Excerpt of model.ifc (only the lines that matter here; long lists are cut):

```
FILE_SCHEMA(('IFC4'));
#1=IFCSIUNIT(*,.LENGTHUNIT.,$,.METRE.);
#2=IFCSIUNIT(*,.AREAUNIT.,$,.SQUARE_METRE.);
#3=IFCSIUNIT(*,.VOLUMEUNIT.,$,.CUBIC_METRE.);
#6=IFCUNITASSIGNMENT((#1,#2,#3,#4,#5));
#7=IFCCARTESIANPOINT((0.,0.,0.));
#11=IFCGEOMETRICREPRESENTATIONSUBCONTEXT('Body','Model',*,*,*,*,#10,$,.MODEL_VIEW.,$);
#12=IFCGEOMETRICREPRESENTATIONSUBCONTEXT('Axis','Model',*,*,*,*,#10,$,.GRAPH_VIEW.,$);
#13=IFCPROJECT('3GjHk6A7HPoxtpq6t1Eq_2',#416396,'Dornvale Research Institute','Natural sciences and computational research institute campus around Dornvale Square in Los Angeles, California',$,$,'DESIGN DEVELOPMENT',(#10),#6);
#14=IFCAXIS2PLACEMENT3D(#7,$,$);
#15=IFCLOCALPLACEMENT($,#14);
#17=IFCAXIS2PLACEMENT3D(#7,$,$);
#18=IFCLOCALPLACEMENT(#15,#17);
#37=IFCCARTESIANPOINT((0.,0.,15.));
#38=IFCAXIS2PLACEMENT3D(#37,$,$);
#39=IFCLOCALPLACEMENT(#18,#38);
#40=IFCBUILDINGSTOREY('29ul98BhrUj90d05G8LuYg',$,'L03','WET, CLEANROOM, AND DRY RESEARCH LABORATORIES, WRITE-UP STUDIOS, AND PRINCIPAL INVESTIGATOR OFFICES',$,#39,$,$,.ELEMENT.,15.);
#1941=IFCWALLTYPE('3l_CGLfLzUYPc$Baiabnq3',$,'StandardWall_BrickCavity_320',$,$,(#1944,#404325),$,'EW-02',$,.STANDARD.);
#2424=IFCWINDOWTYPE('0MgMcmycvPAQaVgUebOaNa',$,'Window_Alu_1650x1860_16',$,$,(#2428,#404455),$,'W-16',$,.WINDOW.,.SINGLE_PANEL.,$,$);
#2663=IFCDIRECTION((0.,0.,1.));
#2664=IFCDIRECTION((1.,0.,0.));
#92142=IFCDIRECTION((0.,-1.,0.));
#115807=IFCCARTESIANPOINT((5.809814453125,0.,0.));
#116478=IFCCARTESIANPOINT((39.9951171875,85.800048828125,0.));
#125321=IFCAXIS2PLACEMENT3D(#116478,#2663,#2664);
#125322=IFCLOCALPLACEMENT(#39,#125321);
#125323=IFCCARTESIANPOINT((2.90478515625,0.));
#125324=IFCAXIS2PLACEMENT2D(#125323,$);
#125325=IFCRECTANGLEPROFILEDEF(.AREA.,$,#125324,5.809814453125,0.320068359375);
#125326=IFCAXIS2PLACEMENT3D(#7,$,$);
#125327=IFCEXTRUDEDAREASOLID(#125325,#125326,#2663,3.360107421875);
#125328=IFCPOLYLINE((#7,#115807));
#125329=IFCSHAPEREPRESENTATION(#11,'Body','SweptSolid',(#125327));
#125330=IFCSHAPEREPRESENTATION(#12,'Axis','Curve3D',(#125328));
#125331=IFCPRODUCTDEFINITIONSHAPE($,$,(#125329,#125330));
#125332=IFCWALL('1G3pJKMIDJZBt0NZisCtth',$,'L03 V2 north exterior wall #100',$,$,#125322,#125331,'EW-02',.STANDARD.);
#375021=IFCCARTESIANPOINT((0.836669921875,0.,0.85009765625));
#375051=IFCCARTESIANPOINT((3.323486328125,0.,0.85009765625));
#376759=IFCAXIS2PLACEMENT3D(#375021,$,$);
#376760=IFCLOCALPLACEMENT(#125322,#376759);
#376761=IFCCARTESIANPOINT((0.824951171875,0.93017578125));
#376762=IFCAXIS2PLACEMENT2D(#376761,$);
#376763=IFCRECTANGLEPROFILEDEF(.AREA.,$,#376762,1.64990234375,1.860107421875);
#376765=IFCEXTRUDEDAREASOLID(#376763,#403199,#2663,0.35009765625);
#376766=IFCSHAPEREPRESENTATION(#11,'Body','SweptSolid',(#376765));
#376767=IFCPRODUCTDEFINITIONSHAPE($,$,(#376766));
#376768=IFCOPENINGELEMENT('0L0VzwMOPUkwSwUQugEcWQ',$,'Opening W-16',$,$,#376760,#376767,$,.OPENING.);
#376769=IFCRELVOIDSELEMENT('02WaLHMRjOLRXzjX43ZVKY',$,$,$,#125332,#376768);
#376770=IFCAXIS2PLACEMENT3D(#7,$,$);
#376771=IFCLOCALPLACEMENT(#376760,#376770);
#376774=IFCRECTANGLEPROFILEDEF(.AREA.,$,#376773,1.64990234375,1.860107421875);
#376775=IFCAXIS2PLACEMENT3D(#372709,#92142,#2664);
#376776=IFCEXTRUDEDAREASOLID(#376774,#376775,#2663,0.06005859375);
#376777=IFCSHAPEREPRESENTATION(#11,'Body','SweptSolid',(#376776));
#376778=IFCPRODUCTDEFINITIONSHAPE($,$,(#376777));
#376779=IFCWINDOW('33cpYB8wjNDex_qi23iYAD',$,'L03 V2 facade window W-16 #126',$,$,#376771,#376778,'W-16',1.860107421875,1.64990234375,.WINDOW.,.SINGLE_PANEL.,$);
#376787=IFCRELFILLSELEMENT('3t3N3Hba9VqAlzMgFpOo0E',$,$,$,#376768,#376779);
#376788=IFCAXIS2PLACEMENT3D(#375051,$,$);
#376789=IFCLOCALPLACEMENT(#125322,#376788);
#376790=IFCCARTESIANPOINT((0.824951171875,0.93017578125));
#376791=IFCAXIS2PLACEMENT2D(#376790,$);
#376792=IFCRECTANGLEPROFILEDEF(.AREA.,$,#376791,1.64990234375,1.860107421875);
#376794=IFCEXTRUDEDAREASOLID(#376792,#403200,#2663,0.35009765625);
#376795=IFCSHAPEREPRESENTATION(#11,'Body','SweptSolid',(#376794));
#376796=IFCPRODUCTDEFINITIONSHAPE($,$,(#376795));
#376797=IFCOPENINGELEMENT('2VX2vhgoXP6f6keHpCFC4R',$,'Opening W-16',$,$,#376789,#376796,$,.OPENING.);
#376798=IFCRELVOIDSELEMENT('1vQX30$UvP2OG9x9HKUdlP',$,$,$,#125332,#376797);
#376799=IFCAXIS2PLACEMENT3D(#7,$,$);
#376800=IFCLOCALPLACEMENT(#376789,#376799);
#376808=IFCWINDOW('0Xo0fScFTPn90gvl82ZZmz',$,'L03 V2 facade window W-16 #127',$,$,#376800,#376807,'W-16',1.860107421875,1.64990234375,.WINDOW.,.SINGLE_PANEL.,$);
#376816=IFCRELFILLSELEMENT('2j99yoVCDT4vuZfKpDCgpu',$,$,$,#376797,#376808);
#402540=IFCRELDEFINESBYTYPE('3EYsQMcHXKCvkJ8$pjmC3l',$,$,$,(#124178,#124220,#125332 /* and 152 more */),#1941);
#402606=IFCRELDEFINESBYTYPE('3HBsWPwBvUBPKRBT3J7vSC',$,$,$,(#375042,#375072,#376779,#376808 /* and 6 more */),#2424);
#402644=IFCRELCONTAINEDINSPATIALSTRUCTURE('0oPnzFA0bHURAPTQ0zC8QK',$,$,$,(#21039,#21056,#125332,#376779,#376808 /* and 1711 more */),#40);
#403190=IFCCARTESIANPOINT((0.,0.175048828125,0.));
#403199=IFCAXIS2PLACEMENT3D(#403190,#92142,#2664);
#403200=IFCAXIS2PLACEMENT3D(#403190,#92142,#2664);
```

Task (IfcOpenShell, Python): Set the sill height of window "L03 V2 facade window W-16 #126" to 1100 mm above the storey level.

```python
import numpy as np
import ifcopenshell
import ifcopenshell.api.geometry
import ifcopenshell.geom
import ifcopenshell.util.element
import ifcopenshell.util.placement
import ifcopenshell.util.shape
import ifcopenshell.util.unit

model = ifcopenshell.open("model.ifc")
unit_scale = ifcopenshell.util.unit.calculate_unit_scale(model)

window = model.by_id(376779)
opening = window.FillsVoids[0].RelatingOpeningElement
storey = ifcopenshell.util.element.get_container(window, ifc_class="IfcBuildingStorey")
level = ifcopenshell.util.placement.get_local_placement(storey.ObjectPlacement)[2, 3]

# The opening's origin need not be at the sill, so measure its lowest point.
shape = ifcopenshell.geom.create_shape(ifcopenshell.geom.settings(), opening)
bottom = ifcopenshell.util.shape.get_shape_bottom_elevation(shape, shape.geometry) / unit_scale
dz = level + 1.1 / unit_scale - bottom

shift = np.array([0.0, 0.0, dz])
# The window is placed relative to its opening, so it follows when the opening moves.
matrix = ifcopenshell.util.placement.get_local_placement(opening.ObjectPlacement)
matrix[:3, 3] += shift
ifcopenshell.api.geometry.edit_object_placement(
    model, product=opening, matrix=matrix, is_si=False, should_transform_children=True
)

print(f"moved by {dz * unit_scale:+.3f} m")

model.write("model_updated.ifc")
```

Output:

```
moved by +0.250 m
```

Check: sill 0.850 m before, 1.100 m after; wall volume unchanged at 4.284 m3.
